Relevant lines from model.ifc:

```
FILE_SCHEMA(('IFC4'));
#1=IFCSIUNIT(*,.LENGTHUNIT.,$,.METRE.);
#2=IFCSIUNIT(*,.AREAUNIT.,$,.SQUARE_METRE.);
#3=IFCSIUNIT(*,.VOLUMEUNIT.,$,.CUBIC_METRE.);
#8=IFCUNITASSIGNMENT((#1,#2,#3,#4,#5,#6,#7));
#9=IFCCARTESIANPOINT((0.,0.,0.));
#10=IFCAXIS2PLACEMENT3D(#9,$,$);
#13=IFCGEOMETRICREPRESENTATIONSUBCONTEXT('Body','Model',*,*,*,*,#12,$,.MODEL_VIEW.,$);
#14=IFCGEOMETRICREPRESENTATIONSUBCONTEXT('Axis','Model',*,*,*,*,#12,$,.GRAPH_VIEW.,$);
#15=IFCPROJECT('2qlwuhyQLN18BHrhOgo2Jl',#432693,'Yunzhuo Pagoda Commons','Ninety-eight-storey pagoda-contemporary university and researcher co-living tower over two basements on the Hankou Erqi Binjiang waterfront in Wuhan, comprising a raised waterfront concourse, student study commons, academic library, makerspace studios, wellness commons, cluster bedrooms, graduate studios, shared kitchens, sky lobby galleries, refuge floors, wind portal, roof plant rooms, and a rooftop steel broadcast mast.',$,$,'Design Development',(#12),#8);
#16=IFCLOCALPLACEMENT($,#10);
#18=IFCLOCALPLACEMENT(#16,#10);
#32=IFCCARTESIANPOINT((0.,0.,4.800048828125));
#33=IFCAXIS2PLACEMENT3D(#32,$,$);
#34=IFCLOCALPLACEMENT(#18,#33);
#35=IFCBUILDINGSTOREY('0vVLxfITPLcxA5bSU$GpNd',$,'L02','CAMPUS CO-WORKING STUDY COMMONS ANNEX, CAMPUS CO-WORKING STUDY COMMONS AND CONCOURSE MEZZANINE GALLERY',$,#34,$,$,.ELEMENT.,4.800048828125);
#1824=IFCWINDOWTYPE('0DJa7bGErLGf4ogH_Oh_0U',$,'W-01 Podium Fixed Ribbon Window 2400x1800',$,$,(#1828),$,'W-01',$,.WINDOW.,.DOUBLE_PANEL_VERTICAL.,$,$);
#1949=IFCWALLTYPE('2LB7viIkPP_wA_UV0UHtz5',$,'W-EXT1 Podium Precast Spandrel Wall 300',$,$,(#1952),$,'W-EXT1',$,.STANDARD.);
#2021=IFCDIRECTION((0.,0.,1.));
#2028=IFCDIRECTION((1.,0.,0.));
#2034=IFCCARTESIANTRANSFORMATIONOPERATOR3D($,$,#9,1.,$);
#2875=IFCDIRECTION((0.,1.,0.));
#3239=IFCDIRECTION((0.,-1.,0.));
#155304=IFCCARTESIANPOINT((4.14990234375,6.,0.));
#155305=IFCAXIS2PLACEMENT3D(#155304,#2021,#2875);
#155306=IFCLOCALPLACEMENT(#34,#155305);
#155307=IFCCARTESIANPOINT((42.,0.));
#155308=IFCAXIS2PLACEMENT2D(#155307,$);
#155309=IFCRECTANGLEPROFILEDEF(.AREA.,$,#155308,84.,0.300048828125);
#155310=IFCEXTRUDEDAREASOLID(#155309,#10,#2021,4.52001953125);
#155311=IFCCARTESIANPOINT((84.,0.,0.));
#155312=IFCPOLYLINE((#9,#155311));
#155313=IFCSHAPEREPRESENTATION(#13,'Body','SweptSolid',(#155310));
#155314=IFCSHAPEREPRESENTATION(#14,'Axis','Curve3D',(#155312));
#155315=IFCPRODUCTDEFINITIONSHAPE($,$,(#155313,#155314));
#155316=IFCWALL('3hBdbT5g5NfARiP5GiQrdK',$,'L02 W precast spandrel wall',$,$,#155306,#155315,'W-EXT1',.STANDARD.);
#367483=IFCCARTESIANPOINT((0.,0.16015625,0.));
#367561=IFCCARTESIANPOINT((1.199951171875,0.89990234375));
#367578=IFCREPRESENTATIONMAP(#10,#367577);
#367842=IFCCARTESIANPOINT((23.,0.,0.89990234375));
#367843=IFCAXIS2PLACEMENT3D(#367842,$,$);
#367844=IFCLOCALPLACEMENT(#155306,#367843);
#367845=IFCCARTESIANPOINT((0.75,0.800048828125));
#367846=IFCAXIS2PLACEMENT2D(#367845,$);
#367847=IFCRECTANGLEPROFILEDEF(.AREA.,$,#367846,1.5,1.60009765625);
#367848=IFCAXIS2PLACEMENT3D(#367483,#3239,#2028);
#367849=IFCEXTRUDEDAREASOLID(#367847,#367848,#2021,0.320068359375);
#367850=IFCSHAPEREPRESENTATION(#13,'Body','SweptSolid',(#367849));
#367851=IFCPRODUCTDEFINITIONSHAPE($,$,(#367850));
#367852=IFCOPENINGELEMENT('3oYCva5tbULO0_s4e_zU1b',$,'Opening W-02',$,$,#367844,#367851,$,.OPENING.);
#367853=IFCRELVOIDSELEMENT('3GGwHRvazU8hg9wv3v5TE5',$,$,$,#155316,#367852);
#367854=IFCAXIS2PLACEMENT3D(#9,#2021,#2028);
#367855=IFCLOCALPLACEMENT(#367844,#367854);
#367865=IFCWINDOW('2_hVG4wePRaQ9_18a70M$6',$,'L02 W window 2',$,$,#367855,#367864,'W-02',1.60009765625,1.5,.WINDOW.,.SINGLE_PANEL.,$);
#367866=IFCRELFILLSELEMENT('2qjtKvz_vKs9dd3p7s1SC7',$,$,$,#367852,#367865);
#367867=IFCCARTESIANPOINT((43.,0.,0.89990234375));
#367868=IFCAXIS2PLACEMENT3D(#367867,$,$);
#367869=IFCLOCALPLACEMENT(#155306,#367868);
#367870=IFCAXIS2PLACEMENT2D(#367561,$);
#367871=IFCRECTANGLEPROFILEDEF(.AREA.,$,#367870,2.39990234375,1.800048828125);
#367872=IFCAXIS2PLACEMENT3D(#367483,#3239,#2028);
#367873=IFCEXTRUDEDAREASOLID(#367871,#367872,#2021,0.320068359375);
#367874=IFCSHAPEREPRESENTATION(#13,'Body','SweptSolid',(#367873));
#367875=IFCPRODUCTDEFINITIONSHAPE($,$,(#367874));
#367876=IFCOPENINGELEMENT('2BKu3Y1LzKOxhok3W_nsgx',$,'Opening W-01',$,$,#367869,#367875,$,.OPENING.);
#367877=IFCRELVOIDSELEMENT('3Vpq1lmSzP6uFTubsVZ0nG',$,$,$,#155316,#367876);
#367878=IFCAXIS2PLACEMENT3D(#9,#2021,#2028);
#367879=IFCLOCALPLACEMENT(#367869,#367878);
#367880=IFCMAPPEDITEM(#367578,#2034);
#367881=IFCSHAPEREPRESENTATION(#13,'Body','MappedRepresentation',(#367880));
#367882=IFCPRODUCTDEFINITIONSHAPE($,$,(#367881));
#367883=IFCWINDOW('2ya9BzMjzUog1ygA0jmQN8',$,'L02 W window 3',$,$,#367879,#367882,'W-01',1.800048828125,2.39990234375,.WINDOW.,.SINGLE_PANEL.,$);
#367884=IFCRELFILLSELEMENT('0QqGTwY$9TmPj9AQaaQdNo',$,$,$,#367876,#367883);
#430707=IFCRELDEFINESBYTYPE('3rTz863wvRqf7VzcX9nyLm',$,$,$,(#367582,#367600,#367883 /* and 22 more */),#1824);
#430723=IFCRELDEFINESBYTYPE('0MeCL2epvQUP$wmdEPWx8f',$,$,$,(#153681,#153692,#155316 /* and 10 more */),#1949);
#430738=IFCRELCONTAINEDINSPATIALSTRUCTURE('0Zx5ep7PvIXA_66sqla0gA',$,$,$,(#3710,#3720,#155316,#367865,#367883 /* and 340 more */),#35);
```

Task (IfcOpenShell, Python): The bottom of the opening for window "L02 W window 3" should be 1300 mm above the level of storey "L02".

```python
import numpy as np
import ifcopenshell
import ifcopenshell.api.geometry
import ifcopenshell.geom
import ifcopenshell.util.element
import ifcopenshell.util.placement
import ifcopenshell.util.shape
import ifcopenshell.util.unit

model = ifcopenshell.open("model.ifc")
unit_scale = ifcopenshell.util.unit.calculate_unit_scale(model)

window = model.by_guid("2ya9BzMjzUog1ygA0jmQN8")
opening = window.FillsVoids[0].RelatingOpeningElement
storey = ifcopenshell.util.element.get_container(window, ifc_class="IfcBuildingStorey")
level = ifcopenshell.util.placement.get_local_placement(storey.ObjectPlacement)[2, 3]

# The opening's origin need not be at the sill, so measure its lowest point.
shape = ifcopenshell.geom.create_shape(ifcopenshell.geom.settings(), opening)
bottom = ifcopenshell.util.shape.get_shape_bottom_elevation(shape, shape.geometry) / unit_scale
dz = level + 1.3 / unit_scale - bottom

shift = np.array([0.0, 0.0, dz])
# The window is placed relative to its opening, so it follows when the opening moves.
matrix = ifcopenshell.util.placement.get_local_placement(opening.ObjectPlacement)
matrix[:3, 3] += shift
ifcopenshell.api.geometry.edit_object_placement(
    model, product=opening, matrix=matrix, is_si=False, should_transform_children=True
)

print(f"moved by {dz * unit_scale:+.3f} m")

model.write("model_edited.ifc")
```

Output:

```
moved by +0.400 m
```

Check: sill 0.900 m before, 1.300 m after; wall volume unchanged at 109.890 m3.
